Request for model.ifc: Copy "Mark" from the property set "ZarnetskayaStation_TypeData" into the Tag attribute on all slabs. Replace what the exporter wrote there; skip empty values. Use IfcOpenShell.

First a look at what the model holds.

```python
import ifcopenshell
import ifcopenshell.util.element

model = ifcopenshell.open("model.ifc")
print(model.schema)
slabs = model.by_type("IfcSlab")
print(len(slabs), "slabs")
for e in slabs[:8]:
    source = ifcopenshell.util.element.get_pset(e, "ZarnetskayaStation_TypeData", "Mark")
    target = e.Tag
    print(e.id(), repr(source), repr(target), sep=" | ")
```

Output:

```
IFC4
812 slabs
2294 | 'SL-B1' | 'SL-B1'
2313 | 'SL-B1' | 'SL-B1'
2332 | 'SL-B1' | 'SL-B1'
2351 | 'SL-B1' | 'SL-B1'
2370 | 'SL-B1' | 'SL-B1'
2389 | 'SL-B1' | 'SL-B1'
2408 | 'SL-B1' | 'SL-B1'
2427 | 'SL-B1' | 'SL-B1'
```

```python
import ifcopenshell
import ifcopenshell.util.element

model = ifcopenshell.open("model.ifc")

count = 0
for e in model.by_type("IfcSlab"):
    value = ifcopenshell.util.element.get_pset(e, "ZarnetskayaStation_TypeData", "Mark")
    current = e.Tag
    if not value or not value.strip() or current == value:
        continue
    e.Tag = value
    count += 1

print(count, "slabs updated")

model.write("model_updated.ifc")
```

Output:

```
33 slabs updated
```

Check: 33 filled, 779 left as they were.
